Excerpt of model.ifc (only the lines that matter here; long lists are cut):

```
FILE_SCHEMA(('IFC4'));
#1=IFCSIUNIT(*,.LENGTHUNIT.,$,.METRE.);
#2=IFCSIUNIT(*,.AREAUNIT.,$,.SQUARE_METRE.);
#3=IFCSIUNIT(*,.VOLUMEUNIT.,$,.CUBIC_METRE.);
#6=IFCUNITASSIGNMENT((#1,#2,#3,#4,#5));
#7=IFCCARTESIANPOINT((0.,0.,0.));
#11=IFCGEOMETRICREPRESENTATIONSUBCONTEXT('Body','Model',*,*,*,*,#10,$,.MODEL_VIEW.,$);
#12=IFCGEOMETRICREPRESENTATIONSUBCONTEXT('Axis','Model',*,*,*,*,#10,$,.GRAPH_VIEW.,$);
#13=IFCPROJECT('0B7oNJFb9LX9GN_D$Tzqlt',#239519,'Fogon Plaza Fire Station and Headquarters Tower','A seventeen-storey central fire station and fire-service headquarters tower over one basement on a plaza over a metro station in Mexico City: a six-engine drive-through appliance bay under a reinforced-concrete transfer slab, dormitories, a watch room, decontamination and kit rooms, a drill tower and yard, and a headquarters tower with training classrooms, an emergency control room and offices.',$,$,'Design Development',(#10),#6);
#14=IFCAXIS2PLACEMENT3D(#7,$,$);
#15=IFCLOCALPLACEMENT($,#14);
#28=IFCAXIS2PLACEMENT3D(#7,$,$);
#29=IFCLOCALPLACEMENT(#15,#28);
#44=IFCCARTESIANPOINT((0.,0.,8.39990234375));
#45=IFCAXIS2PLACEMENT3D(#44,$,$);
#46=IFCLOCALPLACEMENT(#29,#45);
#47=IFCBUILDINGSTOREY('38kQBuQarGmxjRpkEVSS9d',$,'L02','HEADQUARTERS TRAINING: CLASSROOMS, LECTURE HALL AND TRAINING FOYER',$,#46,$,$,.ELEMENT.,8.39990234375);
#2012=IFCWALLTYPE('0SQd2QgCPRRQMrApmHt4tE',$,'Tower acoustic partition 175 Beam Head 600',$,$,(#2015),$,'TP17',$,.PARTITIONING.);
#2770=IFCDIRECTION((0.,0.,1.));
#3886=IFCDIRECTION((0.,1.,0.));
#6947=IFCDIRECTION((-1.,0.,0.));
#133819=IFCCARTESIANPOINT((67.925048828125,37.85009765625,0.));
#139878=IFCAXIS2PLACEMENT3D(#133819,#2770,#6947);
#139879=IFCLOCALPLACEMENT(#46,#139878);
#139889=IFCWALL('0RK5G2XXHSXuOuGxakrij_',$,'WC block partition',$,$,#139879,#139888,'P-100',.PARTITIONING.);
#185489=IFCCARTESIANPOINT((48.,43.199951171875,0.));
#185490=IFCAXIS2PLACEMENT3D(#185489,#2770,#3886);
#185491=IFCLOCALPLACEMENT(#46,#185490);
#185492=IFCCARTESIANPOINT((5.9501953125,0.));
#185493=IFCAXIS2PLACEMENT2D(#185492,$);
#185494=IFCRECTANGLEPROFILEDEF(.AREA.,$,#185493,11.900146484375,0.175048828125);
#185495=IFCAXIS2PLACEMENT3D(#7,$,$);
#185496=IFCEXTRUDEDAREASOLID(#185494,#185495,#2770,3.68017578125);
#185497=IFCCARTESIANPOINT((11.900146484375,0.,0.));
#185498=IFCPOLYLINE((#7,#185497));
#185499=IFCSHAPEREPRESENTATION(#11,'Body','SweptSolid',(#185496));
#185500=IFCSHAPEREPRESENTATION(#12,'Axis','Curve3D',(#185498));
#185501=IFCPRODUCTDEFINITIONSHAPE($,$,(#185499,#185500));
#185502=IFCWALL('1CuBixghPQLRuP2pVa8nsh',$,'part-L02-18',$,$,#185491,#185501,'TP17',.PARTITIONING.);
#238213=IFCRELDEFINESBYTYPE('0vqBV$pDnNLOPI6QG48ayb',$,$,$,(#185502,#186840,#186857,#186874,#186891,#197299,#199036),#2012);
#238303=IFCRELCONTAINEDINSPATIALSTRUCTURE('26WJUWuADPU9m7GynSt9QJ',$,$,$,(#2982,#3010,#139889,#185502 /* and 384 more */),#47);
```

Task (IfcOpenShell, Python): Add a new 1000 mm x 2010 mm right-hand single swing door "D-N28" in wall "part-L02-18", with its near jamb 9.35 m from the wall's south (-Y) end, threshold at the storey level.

```python
import numpy as np
import ifcopenshell
import ifcopenshell.api.feature
import ifcopenshell.api.geometry
import ifcopenshell.api.root
import ifcopenshell.api.spatial
import ifcopenshell.geom
import ifcopenshell.util.element
import ifcopenshell.util.placement
import ifcopenshell.util.representation
import ifcopenshell.util.shape
import ifcopenshell.util.unit

model = ifcopenshell.open("model.ifc")
unit_scale = ifcopenshell.util.unit.calculate_unit_scale(model)
settings = ifcopenshell.geom.settings()


def volume(element):
    """Net volume in cubic metres, openings subtracted."""
    shape = ifcopenshell.geom.create_shape(settings, element)
    return ifcopenshell.util.shape.get_volume(shape.geometry)


wall = model.by_guid("1CuBixghPQLRuP2pVa8nsh")
storey = ifcopenshell.util.element.get_container(wall, ifc_class="IfcBuildingStorey")
context = ifcopenshell.util.representation.get_context(model, "Model", "Body", "MODEL_VIEW")
before = volume(wall)

width, height, from_end, sill = 1, 2.01, 9.35, 0.0  # metres

# The wall runs along its own X axis, and the end named is its -X end.
wall_shape = ifcopenshell.geom.create_shape(settings, wall)
x, y, z = ifcopenshell.util.shape.get_vertices(wall_shape.geometry).T
start = x.min() + from_end
face, thickness = float(y.min()), float(y.max() - y.min())
wall_matrix = ifcopenshell.util.placement.get_local_placement(wall.ObjectPlacement)
level = ifcopenshell.util.placement.get_local_placement(storey.ObjectPlacement)[2, 3]


def in_wall(x, y):
    """Placement at x, y metres in the wall's axes, at sill height."""
    matrix = wall_matrix.copy()
    matrix[:, 3] = wall_matrix @ np.array([x / unit_scale, y / unit_scale, 0.0, 1.0])
    matrix[2, 3] = level + sill / unit_scale
    return matrix


# Opening: a box that overshoots both wall faces by 50 mm.
opening = ifcopenshell.api.root.create_entity(model, ifc_class="IfcOpeningElement", predefined_type="OPENING")
box = ifcopenshell.api.geometry.add_wall_representation(
    model, context=context, length=width, height=height, thickness=thickness + 0.1
)
ifcopenshell.api.geometry.assign_representation(model, product=opening, representation=box)
ifcopenshell.api.geometry.edit_object_placement(model, product=opening, matrix=in_wall(start, face - 0.05), is_si=False)
ifcopenshell.api.feature.add_feature(model, feature=opening, element=wall)

door = ifcopenshell.api.root.create_entity(model, ifc_class="IfcDoor", name="D-N28", predefined_type="DOOR")
door.OverallWidth, door.OverallHeight = width / unit_scale, height / unit_scale
door.OperationType = "SINGLE_SWING_RIGHT"
body = ifcopenshell.api.geometry.add_door_representation(
    model,
    context=context,
    overall_width=door.OverallWidth,
    overall_height=door.OverallHeight,
    operation_type="SINGLE_SWING_RIGHT",
    lining_properties={"LiningDepth": thickness / unit_scale, "ThresholdDepth": thickness / unit_scale},
)
ifcopenshell.api.geometry.assign_representation(model, product=door, representation=body)
ifcopenshell.api.spatial.assign_container(model, products=[door], relating_structure=storey)
ifcopenshell.api.feature.add_filling(model, opening=opening, element=door)

# The lining spans the wall, so the door starts at the wall face.
ifcopenshell.api.geometry.edit_object_placement(model, product=door, matrix=in_wall(start, face), is_si=False)

after = volume(wall)

print(f"wall volume {before:.3f} -> {after:.3f} m3")

model.write("model_updated.ifc")
```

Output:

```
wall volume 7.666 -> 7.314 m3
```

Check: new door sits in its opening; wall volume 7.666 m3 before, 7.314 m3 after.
